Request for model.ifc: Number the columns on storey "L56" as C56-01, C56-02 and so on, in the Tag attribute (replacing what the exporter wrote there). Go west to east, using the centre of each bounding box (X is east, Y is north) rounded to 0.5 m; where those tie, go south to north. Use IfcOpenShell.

First a look at what the model holds.

```python
import ifcopenshell
import ifcopenshell.util.element
import ifcopenshell.util.placement

model = ifcopenshell.open("model.ifc")
print(model.schema)
storey = next(s for s in model.by_type("IfcBuildingStorey") if s.Name == "L56")
columns = [e for e in ifcopenshell.util.element.get_decomposition(storey) if e.is_a("IfcColumn")]
for e in sorted(columns, key=lambda e: e.id()):
    origin = ifcopenshell.util.placement.get_local_placement(e.ObjectPlacement)[:3, 3]
    print(e.id(), e.Tag, e.Name, origin.round(2) + 0.0, sep=" | ")
```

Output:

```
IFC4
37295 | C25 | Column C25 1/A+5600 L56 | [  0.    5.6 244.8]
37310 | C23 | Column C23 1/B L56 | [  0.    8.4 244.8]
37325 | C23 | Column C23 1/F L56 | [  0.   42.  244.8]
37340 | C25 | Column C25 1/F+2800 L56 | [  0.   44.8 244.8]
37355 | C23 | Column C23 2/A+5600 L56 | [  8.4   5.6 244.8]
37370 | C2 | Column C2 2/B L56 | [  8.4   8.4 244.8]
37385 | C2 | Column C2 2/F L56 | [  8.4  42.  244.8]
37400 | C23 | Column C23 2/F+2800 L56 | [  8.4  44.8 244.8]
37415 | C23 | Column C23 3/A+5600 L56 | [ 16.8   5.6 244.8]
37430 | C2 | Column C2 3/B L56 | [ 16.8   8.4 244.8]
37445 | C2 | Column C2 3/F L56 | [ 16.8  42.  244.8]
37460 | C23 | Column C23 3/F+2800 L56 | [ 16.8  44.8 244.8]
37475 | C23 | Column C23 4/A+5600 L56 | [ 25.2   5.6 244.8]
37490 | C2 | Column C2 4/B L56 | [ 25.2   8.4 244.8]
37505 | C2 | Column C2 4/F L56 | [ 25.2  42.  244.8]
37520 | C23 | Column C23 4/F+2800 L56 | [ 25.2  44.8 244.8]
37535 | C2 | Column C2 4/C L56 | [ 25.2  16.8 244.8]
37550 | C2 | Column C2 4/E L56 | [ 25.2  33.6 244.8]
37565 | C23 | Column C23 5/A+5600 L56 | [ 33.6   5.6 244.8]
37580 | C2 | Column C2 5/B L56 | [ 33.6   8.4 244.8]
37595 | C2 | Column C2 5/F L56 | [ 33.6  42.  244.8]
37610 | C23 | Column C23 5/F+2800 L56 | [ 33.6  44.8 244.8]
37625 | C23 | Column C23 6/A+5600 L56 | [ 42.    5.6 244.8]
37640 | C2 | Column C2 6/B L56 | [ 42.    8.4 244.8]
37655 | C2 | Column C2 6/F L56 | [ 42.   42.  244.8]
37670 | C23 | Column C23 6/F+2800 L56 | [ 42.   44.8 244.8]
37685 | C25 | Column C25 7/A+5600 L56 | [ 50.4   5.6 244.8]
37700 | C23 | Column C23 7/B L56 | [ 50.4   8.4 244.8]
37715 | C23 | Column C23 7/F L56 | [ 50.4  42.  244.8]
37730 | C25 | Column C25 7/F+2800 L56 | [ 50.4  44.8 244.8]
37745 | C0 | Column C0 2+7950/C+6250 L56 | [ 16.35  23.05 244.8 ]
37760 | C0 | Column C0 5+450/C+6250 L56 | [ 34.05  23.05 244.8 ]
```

```python
import ifcopenshell
import ifcopenshell.geom
import ifcopenshell.util.element
import ifcopenshell.util.shape

model = ifcopenshell.open("model.ifc")
settings = ifcopenshell.geom.settings()
settings.set("use-world-coords", True)


def centre(element):
    shape = ifcopenshell.geom.create_shape(settings, element)
    return ifcopenshell.util.shape.get_bbox_centroid(shape.geometry)


storey = next(s for s in model.by_type("IfcBuildingStorey") if s.Name == "L56")
columns = [e for e in ifcopenshell.util.element.get_decomposition(storey) if e.is_a("IfcColumn")]

# Insertion points can sit at a corner or the storey origin, so sort by the geometry (in metres).
centres = {e: centre(e) for e in columns}
columns.sort(key=lambda e: (round(centres[e][0] / 0.5), centres[e][1]))

for i, e in enumerate(columns, start=1):
    number = f"C56-{i:02d}"
    e.Tag = number
    print(e.id(), number)

model.write("model_edited.ifc")
```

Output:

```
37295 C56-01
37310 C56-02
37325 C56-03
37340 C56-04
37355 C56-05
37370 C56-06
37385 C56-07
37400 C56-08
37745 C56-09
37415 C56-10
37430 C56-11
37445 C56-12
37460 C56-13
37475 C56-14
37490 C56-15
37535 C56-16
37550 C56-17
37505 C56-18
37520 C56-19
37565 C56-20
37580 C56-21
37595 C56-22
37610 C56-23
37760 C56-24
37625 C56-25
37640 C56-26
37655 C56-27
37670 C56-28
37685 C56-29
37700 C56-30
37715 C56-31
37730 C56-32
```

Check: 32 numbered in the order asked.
